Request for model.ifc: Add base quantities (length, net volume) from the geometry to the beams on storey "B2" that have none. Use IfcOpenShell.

First a look at what the model holds.

```python
import ifcopenshell
import ifcopenshell.util.element
import ifcopenshell.util.unit

model = ifcopenshell.open("model.ifc")
print(model.schema)
for unit_type in ("LENGTHUNIT", "AREAUNIT", "VOLUMEUNIT"):
    print(unit_type, ifcopenshell.util.unit.calculate_unit_scale(model, unit_type))
storey = next(s for s in model.by_type("IfcBuildingStorey") if s.Name == "B2")
beams = [e for e in ifcopenshell.util.element.get_decomposition(storey) if e.is_a("IfcBeam")]
for e in sorted(beams, key=lambda e: e.id()):
    print(e.id(), e.is_a(), e.Name, list(ifcopenshell.util.element.get_psets(e, qtos_only=True)), sep=" | ")
```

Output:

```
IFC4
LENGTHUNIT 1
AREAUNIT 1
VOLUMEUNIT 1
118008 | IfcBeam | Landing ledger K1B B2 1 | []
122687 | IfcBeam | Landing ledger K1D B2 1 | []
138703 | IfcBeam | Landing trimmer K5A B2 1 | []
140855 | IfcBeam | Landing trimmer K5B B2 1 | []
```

```python
import ifcopenshell
import ifcopenshell.api.pset
import ifcopenshell.geom
import ifcopenshell.util.element
import ifcopenshell.util.shape
import ifcopenshell.util.unit

model = ifcopenshell.open("model.ifc")
unit_scale = ifcopenshell.util.unit.calculate_unit_scale(model)
volume_scale = ifcopenshell.util.unit.calculate_unit_scale(model, "VOLUMEUNIT")
settings = ifcopenshell.geom.settings()

storey = next(s for s in model.by_type("IfcBuildingStorey") if s.Name == "B2")
beams = [e for e in ifcopenshell.util.element.get_decomposition(storey) if e.is_a("IfcBeam")]

for e in sorted(beams, key=lambda e: e.id()):
    if ifcopenshell.util.element.get_psets(e, qtos_only=True, should_inherit=False):
        continue
    # Geometry comes back in metres, in the element's own axes.
    shape = ifcopenshell.geom.create_shape(settings, e)
    values = {
        "Length": ifcopenshell.util.shape.get_max_xyz(shape.geometry) / unit_scale,
        "NetVolume": ifcopenshell.util.shape.get_volume(shape.geometry) / volume_scale,
    }
    qto = ifcopenshell.api.pset.add_qto(model, product=e, name="Qto_BeamBaseQuantities")
    ifcopenshell.api.pset.edit_qto(model, qto=qto, properties=values)
    print(e.id(), {k: round(v, 3) for k, v in values.items()})

model.write("model_edited.ifc")
```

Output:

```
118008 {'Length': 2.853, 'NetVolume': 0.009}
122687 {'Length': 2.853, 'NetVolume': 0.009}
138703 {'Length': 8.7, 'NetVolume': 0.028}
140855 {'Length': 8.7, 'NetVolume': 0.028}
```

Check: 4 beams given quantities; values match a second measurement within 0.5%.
